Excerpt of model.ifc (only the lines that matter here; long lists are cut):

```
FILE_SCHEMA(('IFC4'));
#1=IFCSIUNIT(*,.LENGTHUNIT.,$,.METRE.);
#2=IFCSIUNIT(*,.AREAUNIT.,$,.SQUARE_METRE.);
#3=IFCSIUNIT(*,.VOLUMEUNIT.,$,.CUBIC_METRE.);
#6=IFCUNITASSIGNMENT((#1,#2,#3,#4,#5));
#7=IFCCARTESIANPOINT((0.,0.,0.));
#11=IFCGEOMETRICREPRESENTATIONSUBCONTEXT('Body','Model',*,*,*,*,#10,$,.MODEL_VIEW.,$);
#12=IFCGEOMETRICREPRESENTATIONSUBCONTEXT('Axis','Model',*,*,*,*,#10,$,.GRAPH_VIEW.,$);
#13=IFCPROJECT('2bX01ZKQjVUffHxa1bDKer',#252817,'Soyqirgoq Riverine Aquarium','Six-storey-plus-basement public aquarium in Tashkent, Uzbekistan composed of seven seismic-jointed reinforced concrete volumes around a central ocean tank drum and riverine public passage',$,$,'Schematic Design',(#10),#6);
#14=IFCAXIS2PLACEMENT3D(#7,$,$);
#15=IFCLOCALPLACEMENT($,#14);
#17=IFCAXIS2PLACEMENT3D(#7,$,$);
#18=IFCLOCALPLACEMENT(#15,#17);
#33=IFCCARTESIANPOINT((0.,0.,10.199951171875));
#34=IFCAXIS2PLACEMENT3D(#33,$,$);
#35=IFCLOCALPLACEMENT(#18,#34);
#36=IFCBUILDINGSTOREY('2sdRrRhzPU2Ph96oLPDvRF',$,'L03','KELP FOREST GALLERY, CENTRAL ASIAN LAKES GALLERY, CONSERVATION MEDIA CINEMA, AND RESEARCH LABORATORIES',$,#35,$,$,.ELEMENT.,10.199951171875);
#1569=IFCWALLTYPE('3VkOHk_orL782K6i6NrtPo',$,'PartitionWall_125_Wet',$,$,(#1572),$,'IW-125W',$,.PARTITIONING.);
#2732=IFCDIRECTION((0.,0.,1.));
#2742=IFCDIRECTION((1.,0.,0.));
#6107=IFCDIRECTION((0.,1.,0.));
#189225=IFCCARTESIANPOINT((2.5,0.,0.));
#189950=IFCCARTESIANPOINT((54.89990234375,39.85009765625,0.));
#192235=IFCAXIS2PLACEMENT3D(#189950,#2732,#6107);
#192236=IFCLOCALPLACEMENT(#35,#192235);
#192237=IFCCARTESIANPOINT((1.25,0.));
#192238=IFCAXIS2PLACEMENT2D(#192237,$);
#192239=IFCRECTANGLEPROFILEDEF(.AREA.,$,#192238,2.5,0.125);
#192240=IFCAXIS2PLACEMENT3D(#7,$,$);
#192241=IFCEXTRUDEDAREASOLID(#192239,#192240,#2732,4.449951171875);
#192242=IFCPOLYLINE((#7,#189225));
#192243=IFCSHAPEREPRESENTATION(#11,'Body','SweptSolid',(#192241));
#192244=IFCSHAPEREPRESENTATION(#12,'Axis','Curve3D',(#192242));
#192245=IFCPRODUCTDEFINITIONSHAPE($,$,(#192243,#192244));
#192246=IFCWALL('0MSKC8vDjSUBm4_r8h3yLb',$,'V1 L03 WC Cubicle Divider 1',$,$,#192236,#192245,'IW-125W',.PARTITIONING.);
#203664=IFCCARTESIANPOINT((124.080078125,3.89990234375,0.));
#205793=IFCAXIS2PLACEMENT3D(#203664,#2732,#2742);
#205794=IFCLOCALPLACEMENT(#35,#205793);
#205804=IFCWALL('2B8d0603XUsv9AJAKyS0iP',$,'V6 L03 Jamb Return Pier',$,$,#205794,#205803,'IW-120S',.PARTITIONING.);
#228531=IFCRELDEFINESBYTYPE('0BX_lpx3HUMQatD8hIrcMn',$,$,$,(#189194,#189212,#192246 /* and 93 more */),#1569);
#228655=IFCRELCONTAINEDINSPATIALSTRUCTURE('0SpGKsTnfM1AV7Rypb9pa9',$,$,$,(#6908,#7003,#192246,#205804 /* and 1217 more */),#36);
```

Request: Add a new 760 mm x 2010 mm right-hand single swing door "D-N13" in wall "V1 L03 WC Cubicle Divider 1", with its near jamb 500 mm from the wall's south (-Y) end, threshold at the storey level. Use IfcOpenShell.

```python
import numpy as np
import ifcopenshell
import ifcopenshell.api.feature
import ifcopenshell.api.geometry
import ifcopenshell.api.root
import ifcopenshell.api.spatial
import ifcopenshell.geom
import ifcopenshell.util.element
import ifcopenshell.util.placement
import ifcopenshell.util.representation
import ifcopenshell.util.shape
import ifcopenshell.util.unit

model = ifcopenshell.open("model.ifc")
unit_scale = ifcopenshell.util.unit.calculate_unit_scale(model)
settings = ifcopenshell.geom.settings()


def volume(element):
    """Net volume in cubic metres, openings subtracted."""
    shape = ifcopenshell.geom.create_shape(settings, element)
    return ifcopenshell.util.shape.get_volume(shape.geometry)


wall = model.by_guid("0MSKC8vDjSUBm4_r8h3yLb")
storey = ifcopenshell.util.element.get_container(wall, ifc_class="IfcBuildingStorey")
context = ifcopenshell.util.representation.get_context(model, "Model", "Body", "MODEL_VIEW")
before = volume(wall)

width, height, from_end, sill = 0.76, 2.01, 0.5, 0.0  # metres

# The wall runs along its own X axis, and the end named is its -X end.
wall_shape = ifcopenshell.geom.create_shape(settings, wall)
x, y, z = ifcopenshell.util.shape.get_vertices(wall_shape.geometry).T
start = x.min() + from_end
face, thickness = float(y.min()), float(y.max() - y.min())
wall_matrix = ifcopenshell.util.placement.get_local_placement(wall.ObjectPlacement)
level = ifcopenshell.util.placement.get_local_placement(storey.ObjectPlacement)[2, 3]


def in_wall(x, y):
    """Placement at x, y metres in the wall's axes, at sill height."""
    matrix = wall_matrix.copy()
    matrix[:, 3] = wall_matrix @ np.array([x / unit_scale, y / unit_scale, 0.0, 1.0])
    matrix[2, 3] = level + sill / unit_scale
    return matrix


# Opening: a box that overshoots both wall faces by 50 mm.
opening = ifcopenshell.api.root.create_entity(model, ifc_class="IfcOpeningElement", predefined_type="OPENING")
box = ifcopenshell.api.geometry.add_wall_representation(
    model, context=context, length=width, height=height, thickness=thickness + 0.1
)
ifcopenshell.api.geometry.assign_representation(model, product=opening, representation=box)
ifcopenshell.api.geometry.edit_object_placement(model, product=opening, matrix=in_wall(start, face - 0.05), is_si=False)
ifcopenshell.api.feature.add_feature(model, feature=opening, element=wall)

door = ifcopenshell.api.root.create_entity(model, ifc_class="IfcDoor", name="D-N13", predefined_type="DOOR")
door.OverallWidth, door.OverallHeight = width / unit_scale, height / unit_scale
door.OperationType = "SINGLE_SWING_RIGHT"
body = ifcopenshell.api.geometry.add_door_representation(
    model,
    context=context,
    overall_width=door.OverallWidth,
    overall_height=door.OverallHeight,
    operation_type="SINGLE_SWING_RIGHT",
    lining_properties={"LiningDepth": thickness / unit_scale, "ThresholdDepth": thickness / unit_scale},
)
ifcopenshell.api.geometry.assign_representation(model, product=door, representation=body)
ifcopenshell.api.spatial.assign_container(model, products=[door], relating_structure=storey)
ifcopenshell.api.feature.add_filling(model, opening=opening, element=door)

# The lining spans the wall, so the door starts at the wall face.
ifcopenshell.api.geometry.edit_object_placement(model, product=door, matrix=in_wall(start, face), is_si=False)

after = volume(wall)

print(f"wall volume {before:.3f} -> {after:.3f} m3")

model.write("model_v2.ifc")
```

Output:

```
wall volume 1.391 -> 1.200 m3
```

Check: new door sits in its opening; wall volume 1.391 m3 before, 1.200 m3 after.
